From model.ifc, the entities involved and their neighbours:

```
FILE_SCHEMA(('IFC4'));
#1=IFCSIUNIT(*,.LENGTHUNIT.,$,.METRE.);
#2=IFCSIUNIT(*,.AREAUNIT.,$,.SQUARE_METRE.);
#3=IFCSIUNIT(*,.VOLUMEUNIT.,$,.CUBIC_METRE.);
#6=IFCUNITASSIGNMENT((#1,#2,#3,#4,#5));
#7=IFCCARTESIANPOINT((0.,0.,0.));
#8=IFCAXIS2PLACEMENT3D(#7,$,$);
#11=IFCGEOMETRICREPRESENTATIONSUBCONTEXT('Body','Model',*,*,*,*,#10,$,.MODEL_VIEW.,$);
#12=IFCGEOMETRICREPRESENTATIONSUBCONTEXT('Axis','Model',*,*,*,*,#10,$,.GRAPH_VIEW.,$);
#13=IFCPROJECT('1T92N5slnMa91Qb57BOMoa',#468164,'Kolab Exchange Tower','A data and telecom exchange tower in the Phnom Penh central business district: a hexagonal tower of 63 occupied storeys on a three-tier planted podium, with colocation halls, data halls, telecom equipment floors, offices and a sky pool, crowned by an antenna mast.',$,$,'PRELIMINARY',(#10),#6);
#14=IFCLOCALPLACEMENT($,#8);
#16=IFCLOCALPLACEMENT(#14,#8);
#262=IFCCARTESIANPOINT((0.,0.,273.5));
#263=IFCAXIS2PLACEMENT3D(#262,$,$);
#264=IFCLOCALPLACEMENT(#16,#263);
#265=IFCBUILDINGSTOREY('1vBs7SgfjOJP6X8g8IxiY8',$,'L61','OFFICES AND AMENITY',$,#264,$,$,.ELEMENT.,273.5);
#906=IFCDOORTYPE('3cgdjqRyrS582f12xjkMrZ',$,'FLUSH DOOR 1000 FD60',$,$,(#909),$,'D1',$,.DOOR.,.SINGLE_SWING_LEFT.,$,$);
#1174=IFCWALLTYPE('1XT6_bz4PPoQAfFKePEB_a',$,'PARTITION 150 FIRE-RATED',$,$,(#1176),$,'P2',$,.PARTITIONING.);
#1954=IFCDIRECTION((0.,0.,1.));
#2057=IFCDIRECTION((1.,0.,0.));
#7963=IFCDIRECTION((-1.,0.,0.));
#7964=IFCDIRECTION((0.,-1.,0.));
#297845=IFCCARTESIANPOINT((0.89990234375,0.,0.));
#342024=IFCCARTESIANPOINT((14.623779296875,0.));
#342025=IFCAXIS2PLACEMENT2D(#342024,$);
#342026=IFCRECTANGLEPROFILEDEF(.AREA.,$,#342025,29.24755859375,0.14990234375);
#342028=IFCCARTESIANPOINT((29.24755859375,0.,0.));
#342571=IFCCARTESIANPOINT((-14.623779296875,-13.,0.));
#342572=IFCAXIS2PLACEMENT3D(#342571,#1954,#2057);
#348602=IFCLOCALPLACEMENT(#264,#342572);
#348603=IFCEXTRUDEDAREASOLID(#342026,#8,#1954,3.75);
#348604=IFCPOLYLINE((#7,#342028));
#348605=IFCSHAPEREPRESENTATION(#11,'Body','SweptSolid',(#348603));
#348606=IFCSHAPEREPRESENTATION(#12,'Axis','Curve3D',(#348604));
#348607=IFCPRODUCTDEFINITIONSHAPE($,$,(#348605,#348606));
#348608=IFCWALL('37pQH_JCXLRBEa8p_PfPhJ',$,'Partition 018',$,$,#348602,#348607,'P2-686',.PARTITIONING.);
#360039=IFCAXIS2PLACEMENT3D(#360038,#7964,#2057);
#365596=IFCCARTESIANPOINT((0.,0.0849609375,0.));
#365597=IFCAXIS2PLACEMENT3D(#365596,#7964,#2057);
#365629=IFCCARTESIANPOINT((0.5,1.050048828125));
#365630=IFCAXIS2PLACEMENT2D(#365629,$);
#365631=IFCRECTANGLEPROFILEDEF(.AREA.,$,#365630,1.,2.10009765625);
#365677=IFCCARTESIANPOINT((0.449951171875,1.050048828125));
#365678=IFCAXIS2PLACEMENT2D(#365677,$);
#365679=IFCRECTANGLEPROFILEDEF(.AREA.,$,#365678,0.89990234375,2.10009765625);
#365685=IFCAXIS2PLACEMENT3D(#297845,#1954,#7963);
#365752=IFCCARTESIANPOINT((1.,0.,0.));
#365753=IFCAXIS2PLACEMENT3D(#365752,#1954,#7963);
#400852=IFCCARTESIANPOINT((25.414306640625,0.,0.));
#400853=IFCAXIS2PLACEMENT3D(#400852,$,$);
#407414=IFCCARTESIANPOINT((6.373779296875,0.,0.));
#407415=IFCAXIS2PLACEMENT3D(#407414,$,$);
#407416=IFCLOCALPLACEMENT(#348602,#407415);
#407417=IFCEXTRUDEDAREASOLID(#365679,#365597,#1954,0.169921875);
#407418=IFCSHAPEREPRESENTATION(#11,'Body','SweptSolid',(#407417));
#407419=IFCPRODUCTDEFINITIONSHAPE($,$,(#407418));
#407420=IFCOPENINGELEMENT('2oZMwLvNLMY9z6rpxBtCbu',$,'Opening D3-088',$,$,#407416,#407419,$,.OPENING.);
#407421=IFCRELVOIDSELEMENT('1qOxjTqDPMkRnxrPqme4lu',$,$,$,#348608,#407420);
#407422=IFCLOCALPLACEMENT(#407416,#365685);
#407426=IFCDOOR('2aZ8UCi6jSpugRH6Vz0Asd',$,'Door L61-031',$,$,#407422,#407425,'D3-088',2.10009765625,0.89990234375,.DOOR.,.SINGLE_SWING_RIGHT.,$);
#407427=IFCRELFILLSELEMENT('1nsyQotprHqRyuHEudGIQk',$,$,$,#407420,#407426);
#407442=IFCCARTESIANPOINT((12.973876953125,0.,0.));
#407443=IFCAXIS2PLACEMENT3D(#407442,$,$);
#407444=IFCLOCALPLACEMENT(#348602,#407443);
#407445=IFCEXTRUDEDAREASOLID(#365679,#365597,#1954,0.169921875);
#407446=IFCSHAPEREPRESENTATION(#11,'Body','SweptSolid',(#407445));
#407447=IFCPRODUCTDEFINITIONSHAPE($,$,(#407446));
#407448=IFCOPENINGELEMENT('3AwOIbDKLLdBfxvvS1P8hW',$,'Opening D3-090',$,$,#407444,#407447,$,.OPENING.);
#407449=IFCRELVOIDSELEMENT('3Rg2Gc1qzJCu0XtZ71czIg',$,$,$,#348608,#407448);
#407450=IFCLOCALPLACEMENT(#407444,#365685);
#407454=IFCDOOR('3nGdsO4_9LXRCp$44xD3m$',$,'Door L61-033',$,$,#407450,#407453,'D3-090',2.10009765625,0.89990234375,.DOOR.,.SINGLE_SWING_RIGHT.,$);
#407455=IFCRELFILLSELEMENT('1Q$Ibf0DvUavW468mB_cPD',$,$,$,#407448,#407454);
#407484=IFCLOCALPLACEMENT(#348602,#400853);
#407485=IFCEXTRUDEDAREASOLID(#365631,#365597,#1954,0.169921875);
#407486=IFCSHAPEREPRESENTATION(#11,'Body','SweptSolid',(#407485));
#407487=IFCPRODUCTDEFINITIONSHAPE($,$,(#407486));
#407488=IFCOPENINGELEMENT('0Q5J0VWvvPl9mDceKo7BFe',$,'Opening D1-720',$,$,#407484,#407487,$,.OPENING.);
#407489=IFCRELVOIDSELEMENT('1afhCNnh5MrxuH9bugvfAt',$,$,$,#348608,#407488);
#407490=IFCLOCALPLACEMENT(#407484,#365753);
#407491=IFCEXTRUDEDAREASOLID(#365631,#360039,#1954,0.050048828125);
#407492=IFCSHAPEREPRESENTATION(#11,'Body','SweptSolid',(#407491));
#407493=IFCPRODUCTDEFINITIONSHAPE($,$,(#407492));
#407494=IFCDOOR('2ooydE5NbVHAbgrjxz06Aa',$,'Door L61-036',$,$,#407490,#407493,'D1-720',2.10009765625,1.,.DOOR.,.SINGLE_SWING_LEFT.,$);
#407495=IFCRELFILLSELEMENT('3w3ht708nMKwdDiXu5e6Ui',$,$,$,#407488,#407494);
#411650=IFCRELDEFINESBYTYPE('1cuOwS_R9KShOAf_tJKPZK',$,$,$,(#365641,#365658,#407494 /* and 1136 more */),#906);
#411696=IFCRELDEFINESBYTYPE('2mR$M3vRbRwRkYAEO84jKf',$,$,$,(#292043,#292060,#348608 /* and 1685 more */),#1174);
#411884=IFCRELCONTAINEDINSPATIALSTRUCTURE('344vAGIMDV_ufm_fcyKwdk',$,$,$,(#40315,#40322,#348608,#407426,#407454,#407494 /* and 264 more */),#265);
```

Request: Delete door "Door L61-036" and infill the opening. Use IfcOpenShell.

```python
import ifcopenshell
import ifcopenshell.api.feature
import ifcopenshell.api.root
import ifcopenshell.geom
import ifcopenshell.util.shape

model = ifcopenshell.open("model.ifc")
settings = ifcopenshell.geom.settings()


def volume(element):
    """Net volume in cubic metres, openings subtracted."""
    shape = ifcopenshell.geom.create_shape(settings, element)
    return ifcopenshell.util.shape.get_volume(shape.geometry)


door = model.by_guid("2ooydE5NbVHAbgrjxz06Aa")
opening = door.FillsVoids[0].RelatingOpeningElement
wall = opening.VoidsElements[0].RelatingBuildingElement
before = volume(wall)

ifcopenshell.api.root.remove_product(model, product=door)
ifcopenshell.api.feature.remove_feature(model, feature=opening)

after = volume(wall)

print(f"wall volume {before:.3f} -> {after:.3f} m3")

model.write("model_rev.ifc")
```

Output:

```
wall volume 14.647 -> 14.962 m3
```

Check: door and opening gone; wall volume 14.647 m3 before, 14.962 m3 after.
